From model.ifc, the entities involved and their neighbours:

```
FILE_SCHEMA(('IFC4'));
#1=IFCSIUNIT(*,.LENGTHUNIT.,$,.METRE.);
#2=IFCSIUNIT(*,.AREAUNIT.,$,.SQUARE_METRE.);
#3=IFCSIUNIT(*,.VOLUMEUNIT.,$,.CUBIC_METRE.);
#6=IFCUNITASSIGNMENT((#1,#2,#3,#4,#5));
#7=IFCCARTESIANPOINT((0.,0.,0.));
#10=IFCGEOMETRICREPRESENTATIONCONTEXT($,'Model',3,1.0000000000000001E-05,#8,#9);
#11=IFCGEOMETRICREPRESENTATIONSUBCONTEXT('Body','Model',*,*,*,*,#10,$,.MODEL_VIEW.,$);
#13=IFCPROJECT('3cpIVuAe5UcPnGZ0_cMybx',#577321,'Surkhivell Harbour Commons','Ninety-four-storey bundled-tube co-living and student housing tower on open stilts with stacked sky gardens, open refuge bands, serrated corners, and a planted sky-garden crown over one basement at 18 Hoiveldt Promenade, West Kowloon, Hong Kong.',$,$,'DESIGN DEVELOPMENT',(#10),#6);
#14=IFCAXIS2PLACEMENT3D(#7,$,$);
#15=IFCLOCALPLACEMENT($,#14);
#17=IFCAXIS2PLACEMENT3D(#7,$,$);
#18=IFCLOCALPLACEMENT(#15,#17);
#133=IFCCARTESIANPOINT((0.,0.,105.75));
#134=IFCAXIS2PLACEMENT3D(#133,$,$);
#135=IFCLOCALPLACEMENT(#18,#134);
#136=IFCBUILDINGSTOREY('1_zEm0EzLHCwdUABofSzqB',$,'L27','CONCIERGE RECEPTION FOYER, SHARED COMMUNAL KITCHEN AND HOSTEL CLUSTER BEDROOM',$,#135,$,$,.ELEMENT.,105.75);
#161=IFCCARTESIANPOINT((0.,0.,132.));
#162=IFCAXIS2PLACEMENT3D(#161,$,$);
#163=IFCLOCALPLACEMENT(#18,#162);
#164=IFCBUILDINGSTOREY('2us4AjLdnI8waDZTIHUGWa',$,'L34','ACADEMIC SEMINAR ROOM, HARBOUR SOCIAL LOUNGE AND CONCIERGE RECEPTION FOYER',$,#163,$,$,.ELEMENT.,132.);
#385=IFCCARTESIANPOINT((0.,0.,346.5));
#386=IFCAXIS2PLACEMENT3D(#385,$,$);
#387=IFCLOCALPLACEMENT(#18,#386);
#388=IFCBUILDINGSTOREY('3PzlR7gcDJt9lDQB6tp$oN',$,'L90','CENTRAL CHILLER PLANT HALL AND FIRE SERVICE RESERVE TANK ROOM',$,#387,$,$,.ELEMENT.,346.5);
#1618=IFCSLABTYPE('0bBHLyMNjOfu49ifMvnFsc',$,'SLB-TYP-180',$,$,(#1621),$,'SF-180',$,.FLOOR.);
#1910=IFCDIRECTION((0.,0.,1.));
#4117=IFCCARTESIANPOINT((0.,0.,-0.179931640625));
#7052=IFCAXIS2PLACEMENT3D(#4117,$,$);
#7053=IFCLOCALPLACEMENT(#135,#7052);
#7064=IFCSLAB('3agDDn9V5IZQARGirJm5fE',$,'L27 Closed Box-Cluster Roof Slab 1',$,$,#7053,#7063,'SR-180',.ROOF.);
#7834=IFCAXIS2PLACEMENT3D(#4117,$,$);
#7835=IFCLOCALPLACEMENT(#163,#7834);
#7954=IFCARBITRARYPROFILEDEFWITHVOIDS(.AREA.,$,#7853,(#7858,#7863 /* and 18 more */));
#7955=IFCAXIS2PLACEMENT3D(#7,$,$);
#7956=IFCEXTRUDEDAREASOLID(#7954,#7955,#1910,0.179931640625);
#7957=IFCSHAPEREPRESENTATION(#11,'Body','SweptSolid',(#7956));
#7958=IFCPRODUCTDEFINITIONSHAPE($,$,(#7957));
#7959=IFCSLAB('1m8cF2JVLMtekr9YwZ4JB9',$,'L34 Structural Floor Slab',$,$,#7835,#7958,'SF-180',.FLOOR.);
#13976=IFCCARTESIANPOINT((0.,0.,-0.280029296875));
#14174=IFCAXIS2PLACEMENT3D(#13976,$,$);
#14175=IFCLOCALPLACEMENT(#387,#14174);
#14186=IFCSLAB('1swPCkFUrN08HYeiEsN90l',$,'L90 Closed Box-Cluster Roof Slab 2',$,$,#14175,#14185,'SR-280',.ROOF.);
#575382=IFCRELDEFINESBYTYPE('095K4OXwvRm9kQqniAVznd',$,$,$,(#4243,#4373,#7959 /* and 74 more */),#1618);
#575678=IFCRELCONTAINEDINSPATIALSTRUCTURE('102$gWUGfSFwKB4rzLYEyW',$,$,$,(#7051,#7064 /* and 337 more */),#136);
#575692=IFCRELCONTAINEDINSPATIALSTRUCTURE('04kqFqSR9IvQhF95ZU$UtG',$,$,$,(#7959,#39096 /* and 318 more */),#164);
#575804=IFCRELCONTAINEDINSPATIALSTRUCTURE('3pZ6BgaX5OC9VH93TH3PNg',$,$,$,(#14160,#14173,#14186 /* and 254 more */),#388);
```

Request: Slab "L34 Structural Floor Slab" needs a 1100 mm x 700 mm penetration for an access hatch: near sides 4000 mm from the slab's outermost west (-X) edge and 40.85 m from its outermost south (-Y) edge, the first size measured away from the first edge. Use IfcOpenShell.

```python
import numpy as np
import ifcopenshell
import ifcopenshell.api.feature
import ifcopenshell.api.geometry
import ifcopenshell.api.root
import ifcopenshell.geom
import ifcopenshell.util.placement
import ifcopenshell.util.representation
import ifcopenshell.util.shape
import ifcopenshell.util.unit

model = ifcopenshell.open("model.ifc")
unit_scale = ifcopenshell.util.unit.calculate_unit_scale(model)
settings = ifcopenshell.geom.settings()


def volume(element):
    """Net volume in cubic metres, openings subtracted."""
    shape = ifcopenshell.geom.create_shape(settings, element)
    return ifcopenshell.util.shape.get_volume(shape.geometry)


slab = model.by_guid("1m8cF2JVLMtekr9YwZ4JB9")
before = volume(slab)

# Extent in the slab's own axes, in metres. The edges named are its -X and -Y sides.
slab_shape = ifcopenshell.geom.create_shape(settings, slab)
vertices = ifcopenshell.util.shape.get_vertices(slab_shape.geometry)
x_min, y_min, bottom = vertices.min(axis=0)
top = vertices[:, 2].max()

opening = ifcopenshell.api.root.create_entity(model, ifc_class="IfcOpeningElement", name="Access hatch opening", predefined_type="OPENING")
context = ifcopenshell.util.representation.get_context(model, "Model", "Body", "MODEL_VIEW")
width, depth = 1.1, 0.7
outline = [(0.0, 0.0), (width, 0.0), (width, depth), (0.0, depth), (0.0, 0.0)]
# Overshoot both faces by 50 mm so the cut is clean.
shape = ifcopenshell.api.geometry.add_slab_representation(
    model, context=context, depth=top - bottom + 0.1, polyline=outline
)
ifcopenshell.api.geometry.assign_representation(model, product=opening, representation=shape)

matrix = ifcopenshell.util.placement.get_local_placement(slab.ObjectPlacement)
matrix[:, 3] = matrix @ np.append(np.array([x_min + 4, y_min + 40.85, bottom - 0.05]) / unit_scale, 1.0)
ifcopenshell.api.geometry.edit_object_placement(model, product=opening, matrix=matrix, is_si=False)
ifcopenshell.api.feature.add_feature(model, feature=opening, element=slab)

after = volume(slab)

print(f"slab volume {before:.3f} -> {after:.3f} m3")

model.write("model_edited.ifc")
```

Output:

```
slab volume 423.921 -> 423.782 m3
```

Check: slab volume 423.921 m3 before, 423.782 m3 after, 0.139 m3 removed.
